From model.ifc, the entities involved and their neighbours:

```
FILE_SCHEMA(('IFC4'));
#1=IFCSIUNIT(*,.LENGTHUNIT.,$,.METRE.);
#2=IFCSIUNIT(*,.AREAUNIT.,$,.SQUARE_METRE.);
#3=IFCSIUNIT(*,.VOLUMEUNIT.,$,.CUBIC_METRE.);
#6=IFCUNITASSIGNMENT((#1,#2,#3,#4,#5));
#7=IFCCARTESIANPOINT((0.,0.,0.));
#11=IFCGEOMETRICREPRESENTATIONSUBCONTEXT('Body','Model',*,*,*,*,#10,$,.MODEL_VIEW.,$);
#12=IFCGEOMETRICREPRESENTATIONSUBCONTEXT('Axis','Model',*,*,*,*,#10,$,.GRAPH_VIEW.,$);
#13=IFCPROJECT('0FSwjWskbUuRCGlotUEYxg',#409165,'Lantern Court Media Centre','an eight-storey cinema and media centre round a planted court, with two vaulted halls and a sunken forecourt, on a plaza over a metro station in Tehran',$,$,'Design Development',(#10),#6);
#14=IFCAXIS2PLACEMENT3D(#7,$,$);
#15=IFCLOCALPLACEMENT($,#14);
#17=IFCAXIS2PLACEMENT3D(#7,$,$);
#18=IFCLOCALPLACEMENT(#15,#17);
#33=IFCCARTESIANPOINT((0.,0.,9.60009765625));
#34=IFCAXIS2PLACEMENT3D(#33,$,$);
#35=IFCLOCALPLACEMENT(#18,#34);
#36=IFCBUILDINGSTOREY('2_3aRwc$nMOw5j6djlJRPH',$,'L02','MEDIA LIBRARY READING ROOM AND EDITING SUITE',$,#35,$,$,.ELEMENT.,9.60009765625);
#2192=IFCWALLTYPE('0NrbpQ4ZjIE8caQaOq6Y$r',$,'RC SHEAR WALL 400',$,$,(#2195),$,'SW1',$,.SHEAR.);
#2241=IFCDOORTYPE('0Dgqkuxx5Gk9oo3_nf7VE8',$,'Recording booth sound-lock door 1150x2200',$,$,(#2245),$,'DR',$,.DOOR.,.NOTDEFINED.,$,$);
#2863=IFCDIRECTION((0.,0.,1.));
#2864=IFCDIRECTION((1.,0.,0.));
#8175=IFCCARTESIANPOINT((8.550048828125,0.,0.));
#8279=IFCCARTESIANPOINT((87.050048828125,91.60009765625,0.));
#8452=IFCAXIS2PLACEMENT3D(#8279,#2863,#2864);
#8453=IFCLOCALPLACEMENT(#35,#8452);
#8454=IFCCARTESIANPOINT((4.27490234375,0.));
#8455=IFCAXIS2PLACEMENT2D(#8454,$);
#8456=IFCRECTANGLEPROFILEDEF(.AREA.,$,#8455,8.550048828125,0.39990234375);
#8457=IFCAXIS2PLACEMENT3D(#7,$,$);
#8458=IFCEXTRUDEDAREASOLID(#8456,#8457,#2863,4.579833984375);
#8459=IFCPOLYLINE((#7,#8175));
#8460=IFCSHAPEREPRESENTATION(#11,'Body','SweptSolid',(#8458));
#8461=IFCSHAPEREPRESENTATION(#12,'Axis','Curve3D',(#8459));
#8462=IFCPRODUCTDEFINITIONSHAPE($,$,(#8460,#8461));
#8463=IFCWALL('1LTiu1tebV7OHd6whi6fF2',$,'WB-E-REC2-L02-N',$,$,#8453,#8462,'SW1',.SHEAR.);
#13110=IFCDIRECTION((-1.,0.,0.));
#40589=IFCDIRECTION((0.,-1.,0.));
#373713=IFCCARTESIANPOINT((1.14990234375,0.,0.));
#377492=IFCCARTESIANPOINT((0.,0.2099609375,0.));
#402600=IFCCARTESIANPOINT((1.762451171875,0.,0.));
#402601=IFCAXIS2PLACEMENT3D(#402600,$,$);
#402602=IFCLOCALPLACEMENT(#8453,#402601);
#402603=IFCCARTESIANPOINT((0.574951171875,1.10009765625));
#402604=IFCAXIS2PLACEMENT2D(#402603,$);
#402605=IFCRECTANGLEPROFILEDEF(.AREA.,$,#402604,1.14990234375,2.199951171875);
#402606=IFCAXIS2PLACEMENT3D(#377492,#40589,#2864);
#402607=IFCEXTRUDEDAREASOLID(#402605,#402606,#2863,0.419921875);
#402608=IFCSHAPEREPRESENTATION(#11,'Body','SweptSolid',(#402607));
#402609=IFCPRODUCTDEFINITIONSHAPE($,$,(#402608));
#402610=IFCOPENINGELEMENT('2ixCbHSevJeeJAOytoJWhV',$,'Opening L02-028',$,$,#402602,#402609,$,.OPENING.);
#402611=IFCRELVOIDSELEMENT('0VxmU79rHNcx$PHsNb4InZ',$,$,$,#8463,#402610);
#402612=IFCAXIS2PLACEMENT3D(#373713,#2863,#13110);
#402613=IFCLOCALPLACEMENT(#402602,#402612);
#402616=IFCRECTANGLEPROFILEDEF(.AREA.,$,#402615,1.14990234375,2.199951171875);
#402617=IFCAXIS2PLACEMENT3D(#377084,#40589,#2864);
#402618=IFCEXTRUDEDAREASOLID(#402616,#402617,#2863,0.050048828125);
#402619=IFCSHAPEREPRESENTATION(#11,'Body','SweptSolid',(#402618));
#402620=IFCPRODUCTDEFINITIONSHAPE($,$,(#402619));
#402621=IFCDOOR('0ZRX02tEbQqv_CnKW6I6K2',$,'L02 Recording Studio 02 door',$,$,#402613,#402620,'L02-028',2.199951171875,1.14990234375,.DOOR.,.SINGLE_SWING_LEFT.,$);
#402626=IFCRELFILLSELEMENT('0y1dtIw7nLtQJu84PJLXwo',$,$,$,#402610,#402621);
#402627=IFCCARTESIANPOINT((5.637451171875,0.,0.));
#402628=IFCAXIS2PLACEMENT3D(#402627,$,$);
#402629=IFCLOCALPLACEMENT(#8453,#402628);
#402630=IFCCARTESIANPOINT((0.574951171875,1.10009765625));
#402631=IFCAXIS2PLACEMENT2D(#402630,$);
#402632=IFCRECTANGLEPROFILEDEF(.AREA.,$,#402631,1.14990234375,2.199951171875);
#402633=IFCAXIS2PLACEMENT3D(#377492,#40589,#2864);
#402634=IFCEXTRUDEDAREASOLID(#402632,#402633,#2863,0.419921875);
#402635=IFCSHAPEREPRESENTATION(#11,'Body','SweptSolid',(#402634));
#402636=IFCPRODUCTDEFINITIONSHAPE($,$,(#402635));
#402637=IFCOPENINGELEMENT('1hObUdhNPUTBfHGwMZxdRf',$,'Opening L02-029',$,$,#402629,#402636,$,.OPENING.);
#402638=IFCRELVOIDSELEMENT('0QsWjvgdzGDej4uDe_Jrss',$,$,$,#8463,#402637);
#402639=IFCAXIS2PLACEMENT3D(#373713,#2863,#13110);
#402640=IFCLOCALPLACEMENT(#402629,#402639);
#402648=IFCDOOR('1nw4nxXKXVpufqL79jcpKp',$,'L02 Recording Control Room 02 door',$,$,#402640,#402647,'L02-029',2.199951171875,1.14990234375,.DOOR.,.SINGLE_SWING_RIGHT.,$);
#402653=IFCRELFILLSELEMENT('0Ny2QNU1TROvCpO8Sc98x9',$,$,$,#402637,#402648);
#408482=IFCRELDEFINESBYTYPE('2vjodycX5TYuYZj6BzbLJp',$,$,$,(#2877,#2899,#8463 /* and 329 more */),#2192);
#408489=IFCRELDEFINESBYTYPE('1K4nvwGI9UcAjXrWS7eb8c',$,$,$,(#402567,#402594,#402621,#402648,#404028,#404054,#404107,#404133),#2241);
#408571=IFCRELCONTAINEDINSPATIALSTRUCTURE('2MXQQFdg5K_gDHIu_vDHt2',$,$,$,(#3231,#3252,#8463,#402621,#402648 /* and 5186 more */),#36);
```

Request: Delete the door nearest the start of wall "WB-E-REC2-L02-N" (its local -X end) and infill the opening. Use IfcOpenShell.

```python
import ifcopenshell
import ifcopenshell.api.feature
import ifcopenshell.api.root
import ifcopenshell.geom
import ifcopenshell.util.shape

model = ifcopenshell.open("model.ifc")
settings = ifcopenshell.geom.settings()


def volume(element):
    """Net volume in cubic metres, openings subtracted."""
    shape = ifcopenshell.geom.create_shape(settings, element)
    return ifcopenshell.util.shape.get_volume(shape.geometry)


door = model.by_guid("0ZRX02tEbQqv_CnKW6I6K2")
opening = door.FillsVoids[0].RelatingOpeningElement
wall = opening.VoidsElements[0].RelatingBuildingElement
before = volume(wall)

ifcopenshell.api.root.remove_product(model, product=door)
ifcopenshell.api.feature.remove_feature(model, feature=opening)

after = volume(wall)

print(f"wall volume {before:.3f} -> {after:.3f} m3")

model.write("model-out.ifc")
```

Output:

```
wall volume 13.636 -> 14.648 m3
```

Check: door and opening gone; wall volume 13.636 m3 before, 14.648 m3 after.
